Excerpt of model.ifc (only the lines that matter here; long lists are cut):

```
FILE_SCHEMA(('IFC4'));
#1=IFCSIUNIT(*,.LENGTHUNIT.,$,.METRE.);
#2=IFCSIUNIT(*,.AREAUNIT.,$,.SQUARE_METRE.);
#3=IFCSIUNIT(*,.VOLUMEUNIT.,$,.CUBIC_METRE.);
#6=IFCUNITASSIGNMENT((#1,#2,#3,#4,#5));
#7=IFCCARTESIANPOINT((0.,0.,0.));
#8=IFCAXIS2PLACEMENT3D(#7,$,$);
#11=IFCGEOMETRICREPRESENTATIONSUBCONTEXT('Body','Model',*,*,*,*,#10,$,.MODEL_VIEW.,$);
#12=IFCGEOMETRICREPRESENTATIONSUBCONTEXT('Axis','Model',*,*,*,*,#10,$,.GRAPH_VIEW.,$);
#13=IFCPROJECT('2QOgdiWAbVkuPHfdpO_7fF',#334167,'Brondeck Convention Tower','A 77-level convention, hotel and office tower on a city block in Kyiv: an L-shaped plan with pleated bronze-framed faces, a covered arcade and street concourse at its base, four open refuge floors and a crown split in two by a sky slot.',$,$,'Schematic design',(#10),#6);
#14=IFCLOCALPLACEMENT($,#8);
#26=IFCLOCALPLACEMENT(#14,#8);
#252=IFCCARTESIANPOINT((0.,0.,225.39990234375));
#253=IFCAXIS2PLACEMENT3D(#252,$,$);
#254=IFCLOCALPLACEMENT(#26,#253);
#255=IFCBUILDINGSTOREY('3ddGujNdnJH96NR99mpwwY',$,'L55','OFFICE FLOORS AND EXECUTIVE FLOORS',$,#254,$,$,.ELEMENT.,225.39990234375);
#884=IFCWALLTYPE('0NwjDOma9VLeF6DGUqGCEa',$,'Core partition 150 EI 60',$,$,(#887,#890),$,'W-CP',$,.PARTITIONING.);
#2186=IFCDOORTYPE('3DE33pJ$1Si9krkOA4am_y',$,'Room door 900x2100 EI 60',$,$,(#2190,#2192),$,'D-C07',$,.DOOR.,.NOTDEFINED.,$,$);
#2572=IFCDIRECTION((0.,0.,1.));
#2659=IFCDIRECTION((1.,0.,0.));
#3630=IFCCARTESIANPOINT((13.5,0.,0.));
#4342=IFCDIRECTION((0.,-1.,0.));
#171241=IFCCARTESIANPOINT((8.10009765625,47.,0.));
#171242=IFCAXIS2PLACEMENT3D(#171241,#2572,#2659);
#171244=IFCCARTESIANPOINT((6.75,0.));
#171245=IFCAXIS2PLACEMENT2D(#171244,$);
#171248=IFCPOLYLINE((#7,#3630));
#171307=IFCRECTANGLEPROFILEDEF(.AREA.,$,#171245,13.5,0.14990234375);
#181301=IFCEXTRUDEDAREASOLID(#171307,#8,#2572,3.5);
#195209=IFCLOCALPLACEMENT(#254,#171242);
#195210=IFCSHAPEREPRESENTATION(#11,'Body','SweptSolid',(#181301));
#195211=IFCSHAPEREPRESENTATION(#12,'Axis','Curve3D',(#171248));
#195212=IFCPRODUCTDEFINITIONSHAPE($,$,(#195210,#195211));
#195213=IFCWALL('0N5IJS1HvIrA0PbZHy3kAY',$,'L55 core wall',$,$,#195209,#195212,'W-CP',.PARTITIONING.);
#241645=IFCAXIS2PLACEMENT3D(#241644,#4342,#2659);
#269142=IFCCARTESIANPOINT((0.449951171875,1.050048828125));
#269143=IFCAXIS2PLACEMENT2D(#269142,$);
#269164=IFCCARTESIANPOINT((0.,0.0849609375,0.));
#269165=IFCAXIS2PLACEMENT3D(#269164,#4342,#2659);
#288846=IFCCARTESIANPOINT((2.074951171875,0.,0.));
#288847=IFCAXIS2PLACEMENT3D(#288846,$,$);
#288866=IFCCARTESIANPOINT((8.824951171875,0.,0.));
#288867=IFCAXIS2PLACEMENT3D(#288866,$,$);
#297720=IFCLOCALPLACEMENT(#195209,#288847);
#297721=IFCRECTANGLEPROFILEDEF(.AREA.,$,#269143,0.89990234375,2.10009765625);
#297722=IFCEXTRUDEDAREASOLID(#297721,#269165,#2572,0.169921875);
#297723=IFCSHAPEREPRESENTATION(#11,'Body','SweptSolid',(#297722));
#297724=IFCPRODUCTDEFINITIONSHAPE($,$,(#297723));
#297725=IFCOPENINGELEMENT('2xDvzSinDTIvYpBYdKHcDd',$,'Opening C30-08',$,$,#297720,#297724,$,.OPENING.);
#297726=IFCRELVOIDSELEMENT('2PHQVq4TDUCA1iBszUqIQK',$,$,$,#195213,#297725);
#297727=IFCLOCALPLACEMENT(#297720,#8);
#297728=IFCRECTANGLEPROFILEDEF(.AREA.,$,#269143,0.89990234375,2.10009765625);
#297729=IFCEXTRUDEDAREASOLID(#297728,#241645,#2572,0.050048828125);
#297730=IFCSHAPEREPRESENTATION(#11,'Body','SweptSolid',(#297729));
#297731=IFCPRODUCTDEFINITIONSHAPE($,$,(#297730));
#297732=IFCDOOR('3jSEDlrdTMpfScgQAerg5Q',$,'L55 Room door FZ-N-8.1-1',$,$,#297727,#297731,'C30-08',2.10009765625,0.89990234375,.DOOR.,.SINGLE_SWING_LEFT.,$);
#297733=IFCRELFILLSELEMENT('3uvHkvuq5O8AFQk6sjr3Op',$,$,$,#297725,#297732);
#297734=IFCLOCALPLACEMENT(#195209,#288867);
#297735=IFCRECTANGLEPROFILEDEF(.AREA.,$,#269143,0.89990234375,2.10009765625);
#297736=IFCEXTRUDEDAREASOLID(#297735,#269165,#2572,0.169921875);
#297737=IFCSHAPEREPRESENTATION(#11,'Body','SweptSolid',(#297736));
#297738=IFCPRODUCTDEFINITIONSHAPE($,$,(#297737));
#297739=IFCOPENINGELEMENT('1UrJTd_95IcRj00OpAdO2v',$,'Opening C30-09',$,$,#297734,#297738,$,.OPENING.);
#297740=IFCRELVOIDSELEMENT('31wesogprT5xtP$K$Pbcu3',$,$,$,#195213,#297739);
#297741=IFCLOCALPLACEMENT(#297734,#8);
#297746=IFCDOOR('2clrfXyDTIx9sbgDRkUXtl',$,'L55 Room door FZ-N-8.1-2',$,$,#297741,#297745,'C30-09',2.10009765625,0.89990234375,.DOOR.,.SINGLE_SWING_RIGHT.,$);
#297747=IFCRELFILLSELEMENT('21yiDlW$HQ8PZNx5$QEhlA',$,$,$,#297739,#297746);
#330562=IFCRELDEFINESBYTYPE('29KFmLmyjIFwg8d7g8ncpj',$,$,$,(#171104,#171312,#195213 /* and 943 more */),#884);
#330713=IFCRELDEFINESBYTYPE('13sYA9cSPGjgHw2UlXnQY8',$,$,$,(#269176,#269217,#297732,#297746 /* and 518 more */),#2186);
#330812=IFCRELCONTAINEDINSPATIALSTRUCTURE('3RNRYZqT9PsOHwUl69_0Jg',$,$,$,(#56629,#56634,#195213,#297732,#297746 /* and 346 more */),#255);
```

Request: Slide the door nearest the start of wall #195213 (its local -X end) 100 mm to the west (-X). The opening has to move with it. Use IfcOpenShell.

```python
import ifcopenshell
import ifcopenshell.api.geometry
import ifcopenshell.util.placement
import ifcopenshell.util.unit

model = ifcopenshell.open("model.ifc")
unit_scale = ifcopenshell.util.unit.calculate_unit_scale(model)

door = model.by_id(297732)
opening = door.FillsVoids[0].RelatingOpeningElement
wall = opening.VoidsElements[0].RelatingBuildingElement

wall_matrix = ifcopenshell.util.placement.get_local_placement(wall.ObjectPlacement)
shift = wall_matrix[:3, 0] * -0.1 / unit_scale
before = ifcopenshell.util.placement.get_local_placement(door.ObjectPlacement)[:3, 3].copy()

# The door is placed relative to its opening, so it follows when the opening moves.
matrix = ifcopenshell.util.placement.get_local_placement(opening.ObjectPlacement)
matrix[:3, 3] += shift
ifcopenshell.api.geometry.edit_object_placement(
    model, product=opening, matrix=matrix, is_si=False, should_transform_children=True
)

after = ifcopenshell.util.placement.get_local_placement(door.ObjectPlacement)[:3, 3]
print("door moved by", (after - before).round(3) + 0.0)

model.write("model_v2.ifc")
```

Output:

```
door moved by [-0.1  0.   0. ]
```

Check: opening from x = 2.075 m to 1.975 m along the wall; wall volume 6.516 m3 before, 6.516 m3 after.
